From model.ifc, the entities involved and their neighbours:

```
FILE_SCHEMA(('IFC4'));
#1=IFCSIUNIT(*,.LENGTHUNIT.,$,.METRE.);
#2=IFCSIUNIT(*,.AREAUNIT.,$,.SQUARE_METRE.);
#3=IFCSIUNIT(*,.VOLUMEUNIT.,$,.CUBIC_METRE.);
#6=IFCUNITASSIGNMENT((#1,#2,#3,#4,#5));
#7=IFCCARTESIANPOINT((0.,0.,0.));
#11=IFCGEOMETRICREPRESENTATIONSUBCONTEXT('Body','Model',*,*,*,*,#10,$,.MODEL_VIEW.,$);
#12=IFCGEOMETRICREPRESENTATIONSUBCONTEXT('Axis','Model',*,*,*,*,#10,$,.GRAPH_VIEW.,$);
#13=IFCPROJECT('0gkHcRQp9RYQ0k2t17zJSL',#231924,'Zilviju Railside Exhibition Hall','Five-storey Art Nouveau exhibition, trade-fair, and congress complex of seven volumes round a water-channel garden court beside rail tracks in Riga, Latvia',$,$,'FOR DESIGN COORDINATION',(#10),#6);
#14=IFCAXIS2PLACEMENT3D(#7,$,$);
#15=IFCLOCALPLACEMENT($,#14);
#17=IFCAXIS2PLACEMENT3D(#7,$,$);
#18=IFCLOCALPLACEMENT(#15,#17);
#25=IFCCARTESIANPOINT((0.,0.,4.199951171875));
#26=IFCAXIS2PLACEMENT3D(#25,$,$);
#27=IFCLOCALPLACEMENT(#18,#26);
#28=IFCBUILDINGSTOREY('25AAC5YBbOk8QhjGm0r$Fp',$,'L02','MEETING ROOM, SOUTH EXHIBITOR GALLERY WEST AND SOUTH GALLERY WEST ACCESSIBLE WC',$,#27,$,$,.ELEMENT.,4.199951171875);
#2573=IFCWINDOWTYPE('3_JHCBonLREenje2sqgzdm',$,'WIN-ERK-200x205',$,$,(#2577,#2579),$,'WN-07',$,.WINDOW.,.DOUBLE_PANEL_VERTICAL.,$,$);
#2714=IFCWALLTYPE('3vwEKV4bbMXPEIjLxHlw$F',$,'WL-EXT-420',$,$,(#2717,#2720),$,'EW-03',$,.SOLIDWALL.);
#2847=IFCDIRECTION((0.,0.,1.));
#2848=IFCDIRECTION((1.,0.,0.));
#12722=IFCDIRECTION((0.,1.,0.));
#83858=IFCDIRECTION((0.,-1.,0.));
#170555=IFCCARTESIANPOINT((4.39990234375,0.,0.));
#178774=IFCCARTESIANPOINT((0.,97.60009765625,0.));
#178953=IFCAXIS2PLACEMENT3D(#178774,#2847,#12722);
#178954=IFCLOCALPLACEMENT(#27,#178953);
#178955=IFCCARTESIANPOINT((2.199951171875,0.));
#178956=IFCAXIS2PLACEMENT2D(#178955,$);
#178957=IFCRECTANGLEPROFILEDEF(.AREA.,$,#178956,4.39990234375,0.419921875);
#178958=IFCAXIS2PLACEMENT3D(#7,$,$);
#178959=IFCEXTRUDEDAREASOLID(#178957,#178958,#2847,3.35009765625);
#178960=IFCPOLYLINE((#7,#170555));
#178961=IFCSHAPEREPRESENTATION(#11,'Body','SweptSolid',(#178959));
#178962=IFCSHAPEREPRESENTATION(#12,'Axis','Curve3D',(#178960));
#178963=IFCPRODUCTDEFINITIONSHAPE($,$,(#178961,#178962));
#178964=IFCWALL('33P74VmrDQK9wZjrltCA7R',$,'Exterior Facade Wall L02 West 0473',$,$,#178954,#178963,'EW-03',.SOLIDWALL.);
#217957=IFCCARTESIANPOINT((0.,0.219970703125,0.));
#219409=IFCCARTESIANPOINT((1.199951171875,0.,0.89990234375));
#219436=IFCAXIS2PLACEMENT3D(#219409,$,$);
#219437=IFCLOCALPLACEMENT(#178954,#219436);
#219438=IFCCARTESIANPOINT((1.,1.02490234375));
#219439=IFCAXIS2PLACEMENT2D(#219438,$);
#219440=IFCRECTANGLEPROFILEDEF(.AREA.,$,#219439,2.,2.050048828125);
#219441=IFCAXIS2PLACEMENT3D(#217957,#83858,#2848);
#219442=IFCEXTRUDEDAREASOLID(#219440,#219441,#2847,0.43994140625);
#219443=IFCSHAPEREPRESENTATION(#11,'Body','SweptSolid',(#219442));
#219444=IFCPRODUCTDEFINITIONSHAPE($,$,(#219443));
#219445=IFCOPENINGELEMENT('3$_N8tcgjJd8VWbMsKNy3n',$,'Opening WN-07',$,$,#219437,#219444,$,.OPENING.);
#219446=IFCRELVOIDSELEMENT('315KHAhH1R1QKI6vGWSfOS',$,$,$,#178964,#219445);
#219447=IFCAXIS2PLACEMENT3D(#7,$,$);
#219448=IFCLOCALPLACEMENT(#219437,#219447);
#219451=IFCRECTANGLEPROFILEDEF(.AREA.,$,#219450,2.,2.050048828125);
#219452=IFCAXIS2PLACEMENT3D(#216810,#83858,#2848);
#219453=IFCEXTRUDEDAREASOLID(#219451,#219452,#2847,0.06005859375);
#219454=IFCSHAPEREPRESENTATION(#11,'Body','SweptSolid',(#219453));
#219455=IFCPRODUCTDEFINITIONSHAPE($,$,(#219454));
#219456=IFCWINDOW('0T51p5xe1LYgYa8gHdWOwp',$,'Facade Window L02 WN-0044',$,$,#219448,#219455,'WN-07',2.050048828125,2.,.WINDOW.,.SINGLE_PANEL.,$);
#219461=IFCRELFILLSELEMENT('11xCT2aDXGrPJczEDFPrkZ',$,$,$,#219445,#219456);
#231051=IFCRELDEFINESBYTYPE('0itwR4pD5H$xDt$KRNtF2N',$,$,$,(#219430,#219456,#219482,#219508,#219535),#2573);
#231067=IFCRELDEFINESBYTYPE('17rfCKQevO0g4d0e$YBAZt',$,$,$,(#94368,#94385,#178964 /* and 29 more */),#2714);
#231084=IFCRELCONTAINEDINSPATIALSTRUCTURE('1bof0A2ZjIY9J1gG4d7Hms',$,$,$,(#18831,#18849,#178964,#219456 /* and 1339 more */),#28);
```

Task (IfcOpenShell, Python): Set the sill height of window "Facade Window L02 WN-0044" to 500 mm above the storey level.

```python
import numpy as np
import ifcopenshell
import ifcopenshell.api.geometry
import ifcopenshell.geom
import ifcopenshell.util.element
import ifcopenshell.util.placement
import ifcopenshell.util.shape
import ifcopenshell.util.unit

model = ifcopenshell.open("model.ifc")
unit_scale = ifcopenshell.util.unit.calculate_unit_scale(model)

window = model.by_guid("0T51p5xe1LYgYa8gHdWOwp")
opening = window.FillsVoids[0].RelatingOpeningElement
storey = ifcopenshell.util.element.get_container(window, ifc_class="IfcBuildingStorey")
level = ifcopenshell.util.placement.get_local_placement(storey.ObjectPlacement)[2, 3]

# The opening's origin need not be at the sill, so measure its lowest point.
shape = ifcopenshell.geom.create_shape(ifcopenshell.geom.settings(), opening)
bottom = ifcopenshell.util.shape.get_shape_bottom_elevation(shape, shape.geometry) / unit_scale
dz = level + 0.5 - bottom

shift = np.array([0.0, 0.0, dz])
# The window is placed relative to its opening, so it follows when the opening moves.
matrix = ifcopenshell.util.placement.get_local_placement(opening.ObjectPlacement)
matrix[:3, 3] += shift
ifcopenshell.api.geometry.edit_object_placement(
    model, product=opening, matrix=matrix, is_si=False, should_transform_children=True
)

print(f"moved by {dz * unit_scale:+.3f} m")

model.write("model_edited.ifc")
```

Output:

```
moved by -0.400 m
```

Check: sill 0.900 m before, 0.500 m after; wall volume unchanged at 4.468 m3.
